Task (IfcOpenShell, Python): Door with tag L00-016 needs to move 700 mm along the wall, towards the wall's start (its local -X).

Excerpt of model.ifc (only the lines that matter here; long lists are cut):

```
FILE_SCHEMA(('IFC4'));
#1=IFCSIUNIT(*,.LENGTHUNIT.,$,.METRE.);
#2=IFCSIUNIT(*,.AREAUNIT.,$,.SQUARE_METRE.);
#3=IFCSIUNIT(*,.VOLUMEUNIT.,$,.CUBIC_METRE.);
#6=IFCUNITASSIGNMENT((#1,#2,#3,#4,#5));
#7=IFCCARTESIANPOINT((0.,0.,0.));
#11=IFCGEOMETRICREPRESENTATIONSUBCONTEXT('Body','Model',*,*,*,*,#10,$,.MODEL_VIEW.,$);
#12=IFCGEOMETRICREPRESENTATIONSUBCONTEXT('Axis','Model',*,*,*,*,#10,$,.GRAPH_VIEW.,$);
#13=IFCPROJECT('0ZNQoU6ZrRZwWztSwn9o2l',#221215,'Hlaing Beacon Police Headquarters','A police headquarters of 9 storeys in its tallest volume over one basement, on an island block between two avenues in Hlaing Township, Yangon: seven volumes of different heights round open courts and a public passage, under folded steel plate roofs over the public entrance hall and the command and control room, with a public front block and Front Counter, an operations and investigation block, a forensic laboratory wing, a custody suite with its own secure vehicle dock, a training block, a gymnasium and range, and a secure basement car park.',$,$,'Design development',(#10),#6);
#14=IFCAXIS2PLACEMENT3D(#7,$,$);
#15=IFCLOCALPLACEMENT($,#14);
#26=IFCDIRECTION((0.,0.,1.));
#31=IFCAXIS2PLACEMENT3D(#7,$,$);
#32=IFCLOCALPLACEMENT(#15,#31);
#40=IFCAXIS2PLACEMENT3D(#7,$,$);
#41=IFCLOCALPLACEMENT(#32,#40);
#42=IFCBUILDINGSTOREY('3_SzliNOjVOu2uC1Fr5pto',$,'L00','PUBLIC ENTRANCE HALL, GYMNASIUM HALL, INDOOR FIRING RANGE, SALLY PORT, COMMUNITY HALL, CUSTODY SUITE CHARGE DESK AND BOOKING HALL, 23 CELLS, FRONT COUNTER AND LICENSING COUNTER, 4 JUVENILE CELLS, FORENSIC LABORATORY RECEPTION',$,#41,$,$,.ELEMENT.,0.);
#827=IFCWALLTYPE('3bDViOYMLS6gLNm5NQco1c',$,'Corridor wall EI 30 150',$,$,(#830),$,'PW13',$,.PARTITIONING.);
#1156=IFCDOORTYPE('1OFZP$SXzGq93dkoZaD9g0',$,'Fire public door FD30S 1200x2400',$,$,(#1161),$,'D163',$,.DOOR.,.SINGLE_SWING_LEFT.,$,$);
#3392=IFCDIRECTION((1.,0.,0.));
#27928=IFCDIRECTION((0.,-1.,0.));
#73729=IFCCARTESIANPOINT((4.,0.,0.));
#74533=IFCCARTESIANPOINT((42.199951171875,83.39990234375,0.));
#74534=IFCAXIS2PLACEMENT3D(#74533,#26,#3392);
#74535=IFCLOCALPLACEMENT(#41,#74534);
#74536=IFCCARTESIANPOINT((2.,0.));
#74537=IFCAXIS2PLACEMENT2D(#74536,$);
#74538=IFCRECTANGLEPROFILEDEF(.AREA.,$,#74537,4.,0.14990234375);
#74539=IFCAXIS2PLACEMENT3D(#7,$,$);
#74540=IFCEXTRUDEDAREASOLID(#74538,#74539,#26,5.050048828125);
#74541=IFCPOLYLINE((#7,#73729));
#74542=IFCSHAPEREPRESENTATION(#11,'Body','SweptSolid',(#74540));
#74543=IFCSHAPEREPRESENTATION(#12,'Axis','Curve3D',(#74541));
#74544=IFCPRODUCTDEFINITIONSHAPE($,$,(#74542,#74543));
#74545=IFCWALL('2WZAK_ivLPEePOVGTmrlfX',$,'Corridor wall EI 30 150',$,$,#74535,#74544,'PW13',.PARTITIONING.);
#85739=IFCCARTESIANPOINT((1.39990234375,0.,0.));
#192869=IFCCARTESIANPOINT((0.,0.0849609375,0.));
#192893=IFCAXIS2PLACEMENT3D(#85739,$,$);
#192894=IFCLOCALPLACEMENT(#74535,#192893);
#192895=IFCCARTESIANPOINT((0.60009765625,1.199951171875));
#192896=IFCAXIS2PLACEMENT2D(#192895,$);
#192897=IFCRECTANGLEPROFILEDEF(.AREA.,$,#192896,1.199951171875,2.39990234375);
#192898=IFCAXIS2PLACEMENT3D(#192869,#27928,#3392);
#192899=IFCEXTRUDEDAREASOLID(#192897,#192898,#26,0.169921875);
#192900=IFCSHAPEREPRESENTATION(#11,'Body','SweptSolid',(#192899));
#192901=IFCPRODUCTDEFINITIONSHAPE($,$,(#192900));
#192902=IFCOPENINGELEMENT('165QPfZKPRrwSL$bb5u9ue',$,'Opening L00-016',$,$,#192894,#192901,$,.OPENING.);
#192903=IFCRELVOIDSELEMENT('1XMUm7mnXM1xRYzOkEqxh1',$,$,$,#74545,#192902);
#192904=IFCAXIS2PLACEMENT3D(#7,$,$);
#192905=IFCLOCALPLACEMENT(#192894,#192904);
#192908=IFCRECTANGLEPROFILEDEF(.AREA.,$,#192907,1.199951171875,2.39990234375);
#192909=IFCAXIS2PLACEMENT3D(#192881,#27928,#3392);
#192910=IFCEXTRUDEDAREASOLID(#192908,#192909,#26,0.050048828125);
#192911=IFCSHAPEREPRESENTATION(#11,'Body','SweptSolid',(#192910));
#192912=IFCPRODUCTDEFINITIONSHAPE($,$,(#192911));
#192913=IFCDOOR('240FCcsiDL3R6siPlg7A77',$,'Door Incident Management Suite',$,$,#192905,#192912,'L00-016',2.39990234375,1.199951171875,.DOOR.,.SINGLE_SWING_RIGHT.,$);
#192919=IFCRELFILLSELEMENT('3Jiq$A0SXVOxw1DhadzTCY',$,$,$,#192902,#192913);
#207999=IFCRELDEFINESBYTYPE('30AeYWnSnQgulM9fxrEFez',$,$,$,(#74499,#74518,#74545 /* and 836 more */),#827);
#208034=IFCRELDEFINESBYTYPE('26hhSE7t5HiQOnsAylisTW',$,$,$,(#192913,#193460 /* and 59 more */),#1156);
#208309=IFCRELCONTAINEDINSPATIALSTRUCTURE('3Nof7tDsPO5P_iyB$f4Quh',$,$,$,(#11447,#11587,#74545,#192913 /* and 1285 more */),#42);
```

```python
import ifcopenshell
import ifcopenshell.api.geometry
import ifcopenshell.util.placement
import ifcopenshell.util.unit

model = ifcopenshell.open("model.ifc")
unit_scale = ifcopenshell.util.unit.calculate_unit_scale(model)

door = model.by_guid("240FCcsiDL3R6siPlg7A77")
opening = door.FillsVoids[0].RelatingOpeningElement
wall = opening.VoidsElements[0].RelatingBuildingElement

wall_matrix = ifcopenshell.util.placement.get_local_placement(wall.ObjectPlacement)
shift = wall_matrix[:3, 0] * -0.7 / unit_scale
before = ifcopenshell.util.placement.get_local_placement(door.ObjectPlacement)[:3, 3].copy()

# The door is placed relative to its opening, so it follows when the opening moves.
matrix = ifcopenshell.util.placement.get_local_placement(opening.ObjectPlacement)
matrix[:3, 3] += shift
ifcopenshell.api.geometry.edit_object_placement(
    model, product=opening, matrix=matrix, is_si=False, should_transform_children=True
)

after = ifcopenshell.util.placement.get_local_placement(door.ObjectPlacement)[:3, 3]
print("door moved by", (after - before).round(3) + 0.0)

model.write("model_updated.ifc")
```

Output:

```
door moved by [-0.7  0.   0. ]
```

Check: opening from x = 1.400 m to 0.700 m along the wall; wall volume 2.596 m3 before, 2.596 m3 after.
